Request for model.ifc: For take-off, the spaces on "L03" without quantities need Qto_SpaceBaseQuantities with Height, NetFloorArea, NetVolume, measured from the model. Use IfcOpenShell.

First a look at what the model holds.

```python
import ifcopenshell
import ifcopenshell.util.element
import ifcopenshell.util.unit

model = ifcopenshell.open("model.ifc")
print(model.schema)
for unit_type in ("LENGTHUNIT", "AREAUNIT", "VOLUMEUNIT"):
    print(unit_type, ifcopenshell.util.unit.calculate_unit_scale(model, unit_type))
storey = next(s for s in model.by_type("IfcBuildingStorey") if s.Name == "L03")
spaces = [e for e in ifcopenshell.util.element.get_decomposition(storey) if e.is_a("IfcSpace")]
for e in sorted(spaces, key=lambda e: e.id()):
    print(e.id(), e.is_a(), e.Name, list(ifcopenshell.util.element.get_psets(e, qtos_only=True)), sep=" | ")
```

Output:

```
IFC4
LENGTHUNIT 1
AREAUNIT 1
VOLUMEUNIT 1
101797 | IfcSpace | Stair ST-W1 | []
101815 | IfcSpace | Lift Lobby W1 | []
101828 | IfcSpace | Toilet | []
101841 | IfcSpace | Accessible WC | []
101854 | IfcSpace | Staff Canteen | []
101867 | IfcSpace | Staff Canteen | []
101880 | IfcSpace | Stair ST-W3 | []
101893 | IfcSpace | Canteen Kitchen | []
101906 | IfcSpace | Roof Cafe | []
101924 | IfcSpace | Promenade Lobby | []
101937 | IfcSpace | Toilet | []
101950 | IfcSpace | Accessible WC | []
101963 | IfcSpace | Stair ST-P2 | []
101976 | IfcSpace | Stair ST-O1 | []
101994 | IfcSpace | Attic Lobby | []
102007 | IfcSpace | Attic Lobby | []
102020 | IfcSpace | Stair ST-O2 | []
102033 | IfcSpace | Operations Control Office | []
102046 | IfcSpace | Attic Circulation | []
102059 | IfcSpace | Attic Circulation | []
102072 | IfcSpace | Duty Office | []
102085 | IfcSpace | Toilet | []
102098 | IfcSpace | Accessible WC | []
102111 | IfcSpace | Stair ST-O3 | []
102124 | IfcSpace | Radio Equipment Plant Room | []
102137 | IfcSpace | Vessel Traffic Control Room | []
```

```python
import ifcopenshell
import ifcopenshell.api.pset
import ifcopenshell.geom
import ifcopenshell.util.element
import ifcopenshell.util.shape
import ifcopenshell.util.unit

model = ifcopenshell.open("model.ifc")
unit_scale = ifcopenshell.util.unit.calculate_unit_scale(model)
area_scale = ifcopenshell.util.unit.calculate_unit_scale(model, "AREAUNIT")
volume_scale = ifcopenshell.util.unit.calculate_unit_scale(model, "VOLUMEUNIT")
settings = ifcopenshell.geom.settings()

storey = next(s for s in model.by_type("IfcBuildingStorey") if s.Name == "L03")
spaces = [e for e in ifcopenshell.util.element.get_decomposition(storey) if e.is_a("IfcSpace")]

for e in sorted(spaces, key=lambda e: e.id()):
    if ifcopenshell.util.element.get_psets(e, qtos_only=True, should_inherit=False):
        continue
    # Geometry comes back in metres, in the element's own axes.
    shape = ifcopenshell.geom.create_shape(settings, e)
    values = {
        "Height": ifcopenshell.util.shape.get_z(shape.geometry) / unit_scale,
        "NetFloorArea": ifcopenshell.util.shape.get_footprint_area(shape.geometry) / area_scale,
        "NetVolume": ifcopenshell.util.shape.get_volume(shape.geometry) / volume_scale,
    }
    qto = ifcopenshell.api.pset.add_qto(model, product=e, name="Qto_SpaceBaseQuantities")
    ifcopenshell.api.pset.edit_qto(model, qto=qto, properties=values)
    print(e.id(), {k: round(v, 3) for k, v in values.items()})

model.write("model_rev.ifc")
```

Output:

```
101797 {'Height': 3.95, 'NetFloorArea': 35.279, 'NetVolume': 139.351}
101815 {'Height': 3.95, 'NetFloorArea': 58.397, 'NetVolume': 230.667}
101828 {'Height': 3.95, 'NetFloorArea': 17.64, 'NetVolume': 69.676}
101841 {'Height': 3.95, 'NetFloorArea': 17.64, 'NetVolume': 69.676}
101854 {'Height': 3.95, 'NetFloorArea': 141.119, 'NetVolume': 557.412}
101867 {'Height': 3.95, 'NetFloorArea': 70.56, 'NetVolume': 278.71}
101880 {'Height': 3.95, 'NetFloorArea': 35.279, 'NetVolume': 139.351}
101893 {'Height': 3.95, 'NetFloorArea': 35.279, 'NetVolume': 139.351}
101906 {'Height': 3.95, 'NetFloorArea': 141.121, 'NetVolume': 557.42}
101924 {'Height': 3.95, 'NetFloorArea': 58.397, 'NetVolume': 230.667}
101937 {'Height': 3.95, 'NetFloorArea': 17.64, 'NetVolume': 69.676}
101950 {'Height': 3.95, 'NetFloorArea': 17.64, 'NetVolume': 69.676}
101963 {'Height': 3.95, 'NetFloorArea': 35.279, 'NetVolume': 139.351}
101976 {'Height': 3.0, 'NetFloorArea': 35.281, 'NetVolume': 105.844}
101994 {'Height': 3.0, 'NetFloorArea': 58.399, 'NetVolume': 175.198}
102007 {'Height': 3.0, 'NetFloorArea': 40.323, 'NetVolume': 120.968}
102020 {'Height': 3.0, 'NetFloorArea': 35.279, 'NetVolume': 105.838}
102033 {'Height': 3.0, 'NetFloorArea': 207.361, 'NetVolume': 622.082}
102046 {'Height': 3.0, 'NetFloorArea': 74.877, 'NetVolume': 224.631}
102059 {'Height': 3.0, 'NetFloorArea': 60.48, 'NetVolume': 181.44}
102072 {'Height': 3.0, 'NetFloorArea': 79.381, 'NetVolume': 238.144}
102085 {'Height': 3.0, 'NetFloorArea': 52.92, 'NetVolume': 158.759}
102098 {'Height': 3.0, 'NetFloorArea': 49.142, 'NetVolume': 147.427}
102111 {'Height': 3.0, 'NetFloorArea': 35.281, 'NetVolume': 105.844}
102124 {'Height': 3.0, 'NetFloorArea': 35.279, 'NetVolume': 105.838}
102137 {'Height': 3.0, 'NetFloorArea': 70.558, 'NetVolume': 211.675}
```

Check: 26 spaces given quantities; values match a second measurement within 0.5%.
